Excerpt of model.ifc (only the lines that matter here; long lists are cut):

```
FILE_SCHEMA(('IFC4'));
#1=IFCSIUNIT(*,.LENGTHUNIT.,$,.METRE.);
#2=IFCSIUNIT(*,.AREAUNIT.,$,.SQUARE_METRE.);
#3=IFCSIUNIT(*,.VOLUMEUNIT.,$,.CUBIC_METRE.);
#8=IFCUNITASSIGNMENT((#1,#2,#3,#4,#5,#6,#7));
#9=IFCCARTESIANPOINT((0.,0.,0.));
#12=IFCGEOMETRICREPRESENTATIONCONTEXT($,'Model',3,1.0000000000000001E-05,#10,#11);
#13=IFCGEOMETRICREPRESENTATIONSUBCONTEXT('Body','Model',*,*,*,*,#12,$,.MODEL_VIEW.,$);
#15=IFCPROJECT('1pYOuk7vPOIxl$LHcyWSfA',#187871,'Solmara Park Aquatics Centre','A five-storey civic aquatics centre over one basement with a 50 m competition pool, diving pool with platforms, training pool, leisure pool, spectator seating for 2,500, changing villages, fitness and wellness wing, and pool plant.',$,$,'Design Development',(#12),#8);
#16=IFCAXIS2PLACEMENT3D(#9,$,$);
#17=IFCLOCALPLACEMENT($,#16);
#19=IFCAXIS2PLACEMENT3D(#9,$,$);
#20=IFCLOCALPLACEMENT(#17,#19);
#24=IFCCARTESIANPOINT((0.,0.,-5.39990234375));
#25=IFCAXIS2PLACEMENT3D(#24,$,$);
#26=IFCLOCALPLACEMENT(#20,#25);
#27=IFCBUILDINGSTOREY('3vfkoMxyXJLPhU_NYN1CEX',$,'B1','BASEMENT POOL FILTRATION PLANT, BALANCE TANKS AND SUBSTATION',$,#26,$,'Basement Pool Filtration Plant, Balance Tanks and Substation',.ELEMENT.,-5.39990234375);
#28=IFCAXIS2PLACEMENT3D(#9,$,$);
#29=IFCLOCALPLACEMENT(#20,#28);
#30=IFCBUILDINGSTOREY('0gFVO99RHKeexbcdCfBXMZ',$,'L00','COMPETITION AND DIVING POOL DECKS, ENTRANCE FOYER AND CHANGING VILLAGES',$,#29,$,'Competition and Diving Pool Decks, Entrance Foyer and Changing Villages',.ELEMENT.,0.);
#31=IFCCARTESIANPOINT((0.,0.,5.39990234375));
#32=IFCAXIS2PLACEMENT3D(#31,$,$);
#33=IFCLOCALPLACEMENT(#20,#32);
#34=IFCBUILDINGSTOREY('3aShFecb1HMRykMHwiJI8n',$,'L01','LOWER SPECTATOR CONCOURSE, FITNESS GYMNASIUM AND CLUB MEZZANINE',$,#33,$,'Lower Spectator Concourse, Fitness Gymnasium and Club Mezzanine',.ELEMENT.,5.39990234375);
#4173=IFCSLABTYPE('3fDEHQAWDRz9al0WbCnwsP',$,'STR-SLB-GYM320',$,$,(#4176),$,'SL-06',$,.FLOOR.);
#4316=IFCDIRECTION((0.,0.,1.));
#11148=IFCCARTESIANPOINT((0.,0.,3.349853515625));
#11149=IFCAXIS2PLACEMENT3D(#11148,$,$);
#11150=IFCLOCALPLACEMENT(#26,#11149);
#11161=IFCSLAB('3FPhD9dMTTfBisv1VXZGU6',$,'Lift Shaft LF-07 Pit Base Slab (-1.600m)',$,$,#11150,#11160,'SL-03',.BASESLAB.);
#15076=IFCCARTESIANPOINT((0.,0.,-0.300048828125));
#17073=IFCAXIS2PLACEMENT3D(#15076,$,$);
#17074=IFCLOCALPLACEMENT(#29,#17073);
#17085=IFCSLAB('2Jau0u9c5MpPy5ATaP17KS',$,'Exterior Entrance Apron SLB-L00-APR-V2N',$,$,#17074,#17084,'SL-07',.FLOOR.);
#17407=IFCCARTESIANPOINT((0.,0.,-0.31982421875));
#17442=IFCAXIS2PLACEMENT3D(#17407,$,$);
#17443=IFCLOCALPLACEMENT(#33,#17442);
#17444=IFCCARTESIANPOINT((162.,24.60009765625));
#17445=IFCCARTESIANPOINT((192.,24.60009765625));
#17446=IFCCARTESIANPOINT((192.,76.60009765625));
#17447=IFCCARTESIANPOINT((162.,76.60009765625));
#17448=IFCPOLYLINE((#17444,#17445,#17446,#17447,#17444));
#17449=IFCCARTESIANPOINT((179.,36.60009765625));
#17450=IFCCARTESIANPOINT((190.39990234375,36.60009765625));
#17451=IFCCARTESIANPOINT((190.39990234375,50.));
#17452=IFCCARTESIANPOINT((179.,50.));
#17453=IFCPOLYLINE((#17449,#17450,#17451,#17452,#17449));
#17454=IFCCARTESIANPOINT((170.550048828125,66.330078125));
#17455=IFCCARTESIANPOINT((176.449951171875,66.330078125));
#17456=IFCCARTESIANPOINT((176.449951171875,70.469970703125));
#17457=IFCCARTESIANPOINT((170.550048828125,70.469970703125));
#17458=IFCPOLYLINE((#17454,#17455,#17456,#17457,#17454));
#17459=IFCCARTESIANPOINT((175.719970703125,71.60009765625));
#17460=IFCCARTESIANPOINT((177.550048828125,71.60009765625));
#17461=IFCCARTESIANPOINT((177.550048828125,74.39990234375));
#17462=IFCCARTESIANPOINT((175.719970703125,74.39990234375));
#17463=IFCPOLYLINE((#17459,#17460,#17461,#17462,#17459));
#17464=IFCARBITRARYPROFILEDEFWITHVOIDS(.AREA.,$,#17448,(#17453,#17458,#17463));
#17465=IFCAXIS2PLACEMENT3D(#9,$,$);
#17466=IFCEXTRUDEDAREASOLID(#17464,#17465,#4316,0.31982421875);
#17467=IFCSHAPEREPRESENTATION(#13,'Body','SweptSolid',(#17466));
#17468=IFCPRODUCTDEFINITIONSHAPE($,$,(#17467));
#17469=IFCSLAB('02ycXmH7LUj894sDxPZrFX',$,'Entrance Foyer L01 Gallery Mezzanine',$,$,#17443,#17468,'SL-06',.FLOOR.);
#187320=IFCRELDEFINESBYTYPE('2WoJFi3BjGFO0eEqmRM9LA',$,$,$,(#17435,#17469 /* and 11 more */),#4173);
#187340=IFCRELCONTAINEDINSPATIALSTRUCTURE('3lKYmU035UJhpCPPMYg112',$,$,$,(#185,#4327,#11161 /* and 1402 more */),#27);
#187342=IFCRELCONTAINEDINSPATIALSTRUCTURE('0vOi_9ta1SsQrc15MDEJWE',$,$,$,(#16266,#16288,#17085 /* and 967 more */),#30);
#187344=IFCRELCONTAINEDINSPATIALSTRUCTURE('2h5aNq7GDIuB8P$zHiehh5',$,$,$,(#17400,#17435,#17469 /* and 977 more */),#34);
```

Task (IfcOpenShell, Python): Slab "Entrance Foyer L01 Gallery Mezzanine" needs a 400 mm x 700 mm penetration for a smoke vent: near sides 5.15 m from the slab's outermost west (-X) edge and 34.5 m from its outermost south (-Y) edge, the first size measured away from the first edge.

```python
import numpy as np
import ifcopenshell
import ifcopenshell.api.feature
import ifcopenshell.api.geometry
import ifcopenshell.api.root
import ifcopenshell.geom
import ifcopenshell.util.placement
import ifcopenshell.util.representation
import ifcopenshell.util.shape
import ifcopenshell.util.unit

model = ifcopenshell.open("model.ifc")
unit_scale = ifcopenshell.util.unit.calculate_unit_scale(model)
settings = ifcopenshell.geom.settings()


def volume(element):
    """Net volume in cubic metres, openings subtracted."""
    shape = ifcopenshell.geom.create_shape(settings, element)
    return ifcopenshell.util.shape.get_volume(shape.geometry)


slab = model.by_guid("02ycXmH7LUj894sDxPZrFX")
before = volume(slab)

# Extent in the slab's own axes, in metres. The edges named are its -X and -Y sides.
slab_shape = ifcopenshell.geom.create_shape(settings, slab)
vertices = ifcopenshell.util.shape.get_vertices(slab_shape.geometry)
x_min, y_min, bottom = vertices.min(axis=0)
top = vertices[:, 2].max()

opening = ifcopenshell.api.root.create_entity(model, ifc_class="IfcOpeningElement", name="Smoke vent opening", predefined_type="OPENING")
context = ifcopenshell.util.representation.get_context(model, "Model", "Body", "MODEL_VIEW")
width, depth = 0.4, 0.7
outline = [(0.0, 0.0), (width, 0.0), (width, depth), (0.0, depth), (0.0, 0.0)]
# Overshoot both faces by 50 mm so the cut is clean.
shape = ifcopenshell.api.geometry.add_slab_representation(
    model, context=context, depth=top - bottom + 0.1, polyline=outline
)
ifcopenshell.api.geometry.assign_representation(model, product=opening, representation=shape)

matrix = ifcopenshell.util.placement.get_local_placement(slab.ObjectPlacement)
matrix[:, 3] = matrix @ np.append(np.array([x_min + 5.15, y_min + 34.5, bottom - 0.05]) / unit_scale, 1.0)
ifcopenshell.api.geometry.edit_object_placement(model, product=opening, matrix=matrix, is_si=False)
ifcopenshell.api.feature.add_feature(model, feature=opening, element=slab)

after = volume(slab)

print(f"slab volume {before:.3f} -> {after:.3f} m3")

model.write("model_edited.ifc")
```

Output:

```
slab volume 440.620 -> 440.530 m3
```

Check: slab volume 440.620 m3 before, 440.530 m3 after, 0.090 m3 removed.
